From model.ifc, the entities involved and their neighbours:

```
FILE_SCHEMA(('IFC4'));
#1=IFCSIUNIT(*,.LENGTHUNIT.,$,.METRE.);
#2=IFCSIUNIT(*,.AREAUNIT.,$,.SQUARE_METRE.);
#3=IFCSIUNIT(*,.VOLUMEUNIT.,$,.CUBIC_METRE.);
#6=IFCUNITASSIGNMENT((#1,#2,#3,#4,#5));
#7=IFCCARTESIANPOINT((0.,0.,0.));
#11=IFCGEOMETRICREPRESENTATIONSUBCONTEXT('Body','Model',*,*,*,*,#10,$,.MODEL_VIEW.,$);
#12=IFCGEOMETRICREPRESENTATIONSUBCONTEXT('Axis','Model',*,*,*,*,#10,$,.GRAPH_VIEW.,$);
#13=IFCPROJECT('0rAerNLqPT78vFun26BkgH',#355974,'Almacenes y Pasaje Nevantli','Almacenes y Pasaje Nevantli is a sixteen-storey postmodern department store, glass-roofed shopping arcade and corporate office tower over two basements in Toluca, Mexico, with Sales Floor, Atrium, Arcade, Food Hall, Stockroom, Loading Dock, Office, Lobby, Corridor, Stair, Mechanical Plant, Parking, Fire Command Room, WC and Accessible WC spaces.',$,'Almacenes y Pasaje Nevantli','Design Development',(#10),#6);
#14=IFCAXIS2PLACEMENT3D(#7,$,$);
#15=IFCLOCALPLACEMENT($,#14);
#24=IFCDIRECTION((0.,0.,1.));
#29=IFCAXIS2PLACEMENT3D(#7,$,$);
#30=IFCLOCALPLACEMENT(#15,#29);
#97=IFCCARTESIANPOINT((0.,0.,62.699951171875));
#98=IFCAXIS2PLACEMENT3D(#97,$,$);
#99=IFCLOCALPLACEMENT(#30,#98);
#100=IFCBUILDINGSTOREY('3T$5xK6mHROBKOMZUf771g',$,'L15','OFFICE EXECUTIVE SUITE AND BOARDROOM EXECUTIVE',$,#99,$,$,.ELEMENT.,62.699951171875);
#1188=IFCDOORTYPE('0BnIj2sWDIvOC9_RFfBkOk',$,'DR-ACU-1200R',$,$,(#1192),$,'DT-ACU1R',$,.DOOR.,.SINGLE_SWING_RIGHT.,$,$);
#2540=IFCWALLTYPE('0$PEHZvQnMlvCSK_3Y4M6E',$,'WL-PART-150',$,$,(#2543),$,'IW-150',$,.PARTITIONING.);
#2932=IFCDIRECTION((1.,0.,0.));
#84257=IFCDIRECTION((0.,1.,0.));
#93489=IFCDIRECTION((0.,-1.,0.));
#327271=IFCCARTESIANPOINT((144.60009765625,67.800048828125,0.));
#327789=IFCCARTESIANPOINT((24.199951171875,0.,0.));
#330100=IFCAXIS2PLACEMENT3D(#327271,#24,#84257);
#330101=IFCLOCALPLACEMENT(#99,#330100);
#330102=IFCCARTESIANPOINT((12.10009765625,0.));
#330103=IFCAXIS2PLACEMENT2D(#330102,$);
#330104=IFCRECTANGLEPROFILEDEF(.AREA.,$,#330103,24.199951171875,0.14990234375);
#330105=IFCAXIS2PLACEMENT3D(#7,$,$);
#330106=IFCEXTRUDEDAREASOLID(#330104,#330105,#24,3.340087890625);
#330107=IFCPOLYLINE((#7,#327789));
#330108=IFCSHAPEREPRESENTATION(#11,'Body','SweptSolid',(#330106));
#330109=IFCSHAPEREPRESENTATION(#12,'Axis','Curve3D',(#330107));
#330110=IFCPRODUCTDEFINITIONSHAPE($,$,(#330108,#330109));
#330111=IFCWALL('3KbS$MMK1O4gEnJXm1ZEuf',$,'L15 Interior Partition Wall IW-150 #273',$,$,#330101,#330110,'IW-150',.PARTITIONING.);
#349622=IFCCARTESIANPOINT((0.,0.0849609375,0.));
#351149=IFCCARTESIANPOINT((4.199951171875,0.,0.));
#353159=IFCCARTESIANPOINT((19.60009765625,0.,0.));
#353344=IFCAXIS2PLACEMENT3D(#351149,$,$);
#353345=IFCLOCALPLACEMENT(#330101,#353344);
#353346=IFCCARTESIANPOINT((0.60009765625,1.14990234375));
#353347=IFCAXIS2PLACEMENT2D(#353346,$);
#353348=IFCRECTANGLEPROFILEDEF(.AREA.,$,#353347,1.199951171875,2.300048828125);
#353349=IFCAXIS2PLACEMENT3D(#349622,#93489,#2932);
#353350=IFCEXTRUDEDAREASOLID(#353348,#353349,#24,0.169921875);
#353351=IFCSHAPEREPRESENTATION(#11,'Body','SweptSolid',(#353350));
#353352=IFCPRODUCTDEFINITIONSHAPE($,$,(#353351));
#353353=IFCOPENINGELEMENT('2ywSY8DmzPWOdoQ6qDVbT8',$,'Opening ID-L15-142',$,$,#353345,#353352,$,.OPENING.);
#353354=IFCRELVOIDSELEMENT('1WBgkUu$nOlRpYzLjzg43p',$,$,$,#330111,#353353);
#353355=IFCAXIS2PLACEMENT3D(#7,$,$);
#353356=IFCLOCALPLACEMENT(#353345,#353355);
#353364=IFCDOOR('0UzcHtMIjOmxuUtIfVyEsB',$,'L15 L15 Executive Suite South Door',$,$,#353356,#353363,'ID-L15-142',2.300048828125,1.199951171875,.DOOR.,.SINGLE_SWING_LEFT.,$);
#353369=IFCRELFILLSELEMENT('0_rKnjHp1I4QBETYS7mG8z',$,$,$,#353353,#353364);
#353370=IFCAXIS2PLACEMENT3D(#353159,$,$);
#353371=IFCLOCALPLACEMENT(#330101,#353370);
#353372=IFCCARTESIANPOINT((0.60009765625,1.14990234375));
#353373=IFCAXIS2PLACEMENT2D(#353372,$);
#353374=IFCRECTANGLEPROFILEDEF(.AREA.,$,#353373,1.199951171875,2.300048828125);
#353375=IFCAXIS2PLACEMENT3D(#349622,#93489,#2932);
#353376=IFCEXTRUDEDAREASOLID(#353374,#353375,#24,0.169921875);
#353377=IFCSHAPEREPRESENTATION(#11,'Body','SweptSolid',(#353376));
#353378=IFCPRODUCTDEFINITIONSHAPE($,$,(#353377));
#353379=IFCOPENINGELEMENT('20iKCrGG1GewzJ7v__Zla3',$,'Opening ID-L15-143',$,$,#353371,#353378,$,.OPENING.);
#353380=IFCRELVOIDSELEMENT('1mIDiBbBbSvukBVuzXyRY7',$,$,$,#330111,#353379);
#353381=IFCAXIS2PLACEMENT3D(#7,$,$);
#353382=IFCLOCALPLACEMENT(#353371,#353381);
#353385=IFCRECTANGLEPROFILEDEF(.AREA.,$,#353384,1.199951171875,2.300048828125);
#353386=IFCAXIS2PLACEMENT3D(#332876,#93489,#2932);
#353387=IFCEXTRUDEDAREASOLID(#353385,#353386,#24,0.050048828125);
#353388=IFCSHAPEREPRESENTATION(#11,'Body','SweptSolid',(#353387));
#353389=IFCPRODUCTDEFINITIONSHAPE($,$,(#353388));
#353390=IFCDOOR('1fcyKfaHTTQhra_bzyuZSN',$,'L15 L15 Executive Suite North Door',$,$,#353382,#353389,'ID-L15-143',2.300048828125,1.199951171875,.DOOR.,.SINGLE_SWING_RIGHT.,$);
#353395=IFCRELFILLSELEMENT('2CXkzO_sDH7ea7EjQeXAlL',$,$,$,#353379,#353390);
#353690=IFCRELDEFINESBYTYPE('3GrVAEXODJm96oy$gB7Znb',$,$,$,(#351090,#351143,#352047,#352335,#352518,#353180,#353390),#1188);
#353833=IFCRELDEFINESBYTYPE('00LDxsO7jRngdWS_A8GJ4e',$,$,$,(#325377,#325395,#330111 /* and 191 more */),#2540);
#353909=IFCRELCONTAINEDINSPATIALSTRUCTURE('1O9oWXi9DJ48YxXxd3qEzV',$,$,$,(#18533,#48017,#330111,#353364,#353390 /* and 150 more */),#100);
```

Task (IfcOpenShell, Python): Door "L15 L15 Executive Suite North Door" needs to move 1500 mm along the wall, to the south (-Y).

```python
import ifcopenshell
import ifcopenshell.api.geometry
import ifcopenshell.util.placement

model = ifcopenshell.open("model.ifc")

door = model.by_id(353390)
opening = door.FillsVoids[0].RelatingOpeningElement
wall = opening.VoidsElements[0].RelatingBuildingElement

wall_matrix = ifcopenshell.util.placement.get_local_placement(wall.ObjectPlacement)
shift = wall_matrix[:3, 0] * -1.5
before = ifcopenshell.util.placement.get_local_placement(door.ObjectPlacement)[:3, 3].copy()

# The door is placed relative to its opening, so it follows when the opening moves.
matrix = ifcopenshell.util.placement.get_local_placement(opening.ObjectPlacement)
matrix[:3, 3] += shift
ifcopenshell.api.geometry.edit_object_placement(
    model, product=opening, matrix=matrix, is_si=False, should_transform_children=True
)

after = ifcopenshell.util.placement.get_local_placement(door.ObjectPlacement)[:3, 3]
print("door moved by", (after - before).round(3) + 0.0)

model.write("model_v2.ifc")
```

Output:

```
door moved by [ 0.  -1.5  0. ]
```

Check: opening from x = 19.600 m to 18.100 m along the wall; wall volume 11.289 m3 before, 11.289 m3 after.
